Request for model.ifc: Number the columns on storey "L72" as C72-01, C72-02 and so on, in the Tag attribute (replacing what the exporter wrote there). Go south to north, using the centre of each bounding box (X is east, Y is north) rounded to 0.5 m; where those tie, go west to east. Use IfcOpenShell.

First a look at what the model holds.

```python
import ifcopenshell
import ifcopenshell.util.element
import ifcopenshell.util.placement

model = ifcopenshell.open("model.ifc")
print(model.schema)
storey = next(s for s in model.by_type("IfcBuildingStorey") if s.Name == "L72")
columns = [e for e in ifcopenshell.util.element.get_decomposition(storey) if e.is_a("IfcColumn")]
for e in sorted(columns, key=lambda e: e.id()):
    origin = ifcopenshell.util.placement.get_local_placement(e.ObjectPlacement)[:3, 3]
    print(e.id(), e.Tag, e.Name, origin.round(2) + 0.0, sep=" | ")
```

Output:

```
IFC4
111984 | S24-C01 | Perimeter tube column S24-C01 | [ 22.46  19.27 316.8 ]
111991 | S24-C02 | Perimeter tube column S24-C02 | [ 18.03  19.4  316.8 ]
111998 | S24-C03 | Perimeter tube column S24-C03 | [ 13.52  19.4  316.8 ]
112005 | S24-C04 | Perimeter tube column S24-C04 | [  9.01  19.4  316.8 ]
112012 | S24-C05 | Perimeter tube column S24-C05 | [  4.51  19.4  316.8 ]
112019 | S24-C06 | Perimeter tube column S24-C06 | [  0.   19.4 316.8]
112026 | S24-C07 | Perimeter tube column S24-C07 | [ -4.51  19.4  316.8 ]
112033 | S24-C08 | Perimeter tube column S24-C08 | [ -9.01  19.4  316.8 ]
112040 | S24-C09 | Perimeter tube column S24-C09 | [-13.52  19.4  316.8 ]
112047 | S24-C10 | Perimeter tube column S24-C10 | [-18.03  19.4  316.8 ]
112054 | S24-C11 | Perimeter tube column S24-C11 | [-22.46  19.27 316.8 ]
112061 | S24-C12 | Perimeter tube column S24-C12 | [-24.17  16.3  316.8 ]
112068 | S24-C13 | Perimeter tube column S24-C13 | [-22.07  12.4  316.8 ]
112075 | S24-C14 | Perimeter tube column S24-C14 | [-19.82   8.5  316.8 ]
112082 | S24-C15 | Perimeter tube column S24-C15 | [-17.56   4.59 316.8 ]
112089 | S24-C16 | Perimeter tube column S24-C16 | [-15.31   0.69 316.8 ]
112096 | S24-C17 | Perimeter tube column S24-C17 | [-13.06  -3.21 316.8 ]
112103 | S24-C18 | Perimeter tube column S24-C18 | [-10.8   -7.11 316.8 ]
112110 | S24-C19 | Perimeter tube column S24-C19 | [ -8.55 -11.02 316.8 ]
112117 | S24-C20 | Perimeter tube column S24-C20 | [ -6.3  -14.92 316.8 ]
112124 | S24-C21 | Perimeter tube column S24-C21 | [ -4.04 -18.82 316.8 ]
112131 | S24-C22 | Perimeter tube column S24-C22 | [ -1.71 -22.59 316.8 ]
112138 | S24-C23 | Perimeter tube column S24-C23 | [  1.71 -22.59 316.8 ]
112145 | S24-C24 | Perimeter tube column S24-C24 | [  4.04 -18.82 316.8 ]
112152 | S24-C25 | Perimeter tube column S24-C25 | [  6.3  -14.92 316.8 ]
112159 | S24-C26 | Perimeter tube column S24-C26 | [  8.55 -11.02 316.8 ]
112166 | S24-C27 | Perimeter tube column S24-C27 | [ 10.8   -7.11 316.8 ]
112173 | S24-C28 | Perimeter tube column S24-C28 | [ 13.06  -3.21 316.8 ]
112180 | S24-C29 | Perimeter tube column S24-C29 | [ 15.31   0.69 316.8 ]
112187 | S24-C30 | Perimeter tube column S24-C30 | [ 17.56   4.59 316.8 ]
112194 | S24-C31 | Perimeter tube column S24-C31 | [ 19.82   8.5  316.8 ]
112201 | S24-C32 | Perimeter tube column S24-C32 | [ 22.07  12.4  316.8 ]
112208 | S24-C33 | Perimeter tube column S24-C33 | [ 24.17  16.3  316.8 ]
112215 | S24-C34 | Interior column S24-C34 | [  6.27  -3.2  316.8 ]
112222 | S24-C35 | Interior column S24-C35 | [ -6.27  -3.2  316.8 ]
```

```python
import ifcopenshell
import ifcopenshell.geom
import ifcopenshell.util.element
import ifcopenshell.util.shape

model = ifcopenshell.open("model.ifc")
settings = ifcopenshell.geom.settings()
settings.set("use-world-coords", True)


def centre(element):
    shape = ifcopenshell.geom.create_shape(settings, element)
    return ifcopenshell.util.shape.get_bbox_centroid(shape.geometry)


storey = next(s for s in model.by_type("IfcBuildingStorey") if s.Name == "L72")
columns = [e for e in ifcopenshell.util.element.get_decomposition(storey) if e.is_a("IfcColumn")]

# Insertion points can sit at a corner or the storey origin, so sort by the geometry (in metres).
centres = {e: centre(e) for e in columns}
columns.sort(key=lambda e: (round(centres[e][1] / 0.5), centres[e][0]))

for i, e in enumerate(columns, start=1):
    number = f"C72-{i:02d}"
    e.Tag = number
    print(e.id(), number)

model.write("model_edited.ifc")
```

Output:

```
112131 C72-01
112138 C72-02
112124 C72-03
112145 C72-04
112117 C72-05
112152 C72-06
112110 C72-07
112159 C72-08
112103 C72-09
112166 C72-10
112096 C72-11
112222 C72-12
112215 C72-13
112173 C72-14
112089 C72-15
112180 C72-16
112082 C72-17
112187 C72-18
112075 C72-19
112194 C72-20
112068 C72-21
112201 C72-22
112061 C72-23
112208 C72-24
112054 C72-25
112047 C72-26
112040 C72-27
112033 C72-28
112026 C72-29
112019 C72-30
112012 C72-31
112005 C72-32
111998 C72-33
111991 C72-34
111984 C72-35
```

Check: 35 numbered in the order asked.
